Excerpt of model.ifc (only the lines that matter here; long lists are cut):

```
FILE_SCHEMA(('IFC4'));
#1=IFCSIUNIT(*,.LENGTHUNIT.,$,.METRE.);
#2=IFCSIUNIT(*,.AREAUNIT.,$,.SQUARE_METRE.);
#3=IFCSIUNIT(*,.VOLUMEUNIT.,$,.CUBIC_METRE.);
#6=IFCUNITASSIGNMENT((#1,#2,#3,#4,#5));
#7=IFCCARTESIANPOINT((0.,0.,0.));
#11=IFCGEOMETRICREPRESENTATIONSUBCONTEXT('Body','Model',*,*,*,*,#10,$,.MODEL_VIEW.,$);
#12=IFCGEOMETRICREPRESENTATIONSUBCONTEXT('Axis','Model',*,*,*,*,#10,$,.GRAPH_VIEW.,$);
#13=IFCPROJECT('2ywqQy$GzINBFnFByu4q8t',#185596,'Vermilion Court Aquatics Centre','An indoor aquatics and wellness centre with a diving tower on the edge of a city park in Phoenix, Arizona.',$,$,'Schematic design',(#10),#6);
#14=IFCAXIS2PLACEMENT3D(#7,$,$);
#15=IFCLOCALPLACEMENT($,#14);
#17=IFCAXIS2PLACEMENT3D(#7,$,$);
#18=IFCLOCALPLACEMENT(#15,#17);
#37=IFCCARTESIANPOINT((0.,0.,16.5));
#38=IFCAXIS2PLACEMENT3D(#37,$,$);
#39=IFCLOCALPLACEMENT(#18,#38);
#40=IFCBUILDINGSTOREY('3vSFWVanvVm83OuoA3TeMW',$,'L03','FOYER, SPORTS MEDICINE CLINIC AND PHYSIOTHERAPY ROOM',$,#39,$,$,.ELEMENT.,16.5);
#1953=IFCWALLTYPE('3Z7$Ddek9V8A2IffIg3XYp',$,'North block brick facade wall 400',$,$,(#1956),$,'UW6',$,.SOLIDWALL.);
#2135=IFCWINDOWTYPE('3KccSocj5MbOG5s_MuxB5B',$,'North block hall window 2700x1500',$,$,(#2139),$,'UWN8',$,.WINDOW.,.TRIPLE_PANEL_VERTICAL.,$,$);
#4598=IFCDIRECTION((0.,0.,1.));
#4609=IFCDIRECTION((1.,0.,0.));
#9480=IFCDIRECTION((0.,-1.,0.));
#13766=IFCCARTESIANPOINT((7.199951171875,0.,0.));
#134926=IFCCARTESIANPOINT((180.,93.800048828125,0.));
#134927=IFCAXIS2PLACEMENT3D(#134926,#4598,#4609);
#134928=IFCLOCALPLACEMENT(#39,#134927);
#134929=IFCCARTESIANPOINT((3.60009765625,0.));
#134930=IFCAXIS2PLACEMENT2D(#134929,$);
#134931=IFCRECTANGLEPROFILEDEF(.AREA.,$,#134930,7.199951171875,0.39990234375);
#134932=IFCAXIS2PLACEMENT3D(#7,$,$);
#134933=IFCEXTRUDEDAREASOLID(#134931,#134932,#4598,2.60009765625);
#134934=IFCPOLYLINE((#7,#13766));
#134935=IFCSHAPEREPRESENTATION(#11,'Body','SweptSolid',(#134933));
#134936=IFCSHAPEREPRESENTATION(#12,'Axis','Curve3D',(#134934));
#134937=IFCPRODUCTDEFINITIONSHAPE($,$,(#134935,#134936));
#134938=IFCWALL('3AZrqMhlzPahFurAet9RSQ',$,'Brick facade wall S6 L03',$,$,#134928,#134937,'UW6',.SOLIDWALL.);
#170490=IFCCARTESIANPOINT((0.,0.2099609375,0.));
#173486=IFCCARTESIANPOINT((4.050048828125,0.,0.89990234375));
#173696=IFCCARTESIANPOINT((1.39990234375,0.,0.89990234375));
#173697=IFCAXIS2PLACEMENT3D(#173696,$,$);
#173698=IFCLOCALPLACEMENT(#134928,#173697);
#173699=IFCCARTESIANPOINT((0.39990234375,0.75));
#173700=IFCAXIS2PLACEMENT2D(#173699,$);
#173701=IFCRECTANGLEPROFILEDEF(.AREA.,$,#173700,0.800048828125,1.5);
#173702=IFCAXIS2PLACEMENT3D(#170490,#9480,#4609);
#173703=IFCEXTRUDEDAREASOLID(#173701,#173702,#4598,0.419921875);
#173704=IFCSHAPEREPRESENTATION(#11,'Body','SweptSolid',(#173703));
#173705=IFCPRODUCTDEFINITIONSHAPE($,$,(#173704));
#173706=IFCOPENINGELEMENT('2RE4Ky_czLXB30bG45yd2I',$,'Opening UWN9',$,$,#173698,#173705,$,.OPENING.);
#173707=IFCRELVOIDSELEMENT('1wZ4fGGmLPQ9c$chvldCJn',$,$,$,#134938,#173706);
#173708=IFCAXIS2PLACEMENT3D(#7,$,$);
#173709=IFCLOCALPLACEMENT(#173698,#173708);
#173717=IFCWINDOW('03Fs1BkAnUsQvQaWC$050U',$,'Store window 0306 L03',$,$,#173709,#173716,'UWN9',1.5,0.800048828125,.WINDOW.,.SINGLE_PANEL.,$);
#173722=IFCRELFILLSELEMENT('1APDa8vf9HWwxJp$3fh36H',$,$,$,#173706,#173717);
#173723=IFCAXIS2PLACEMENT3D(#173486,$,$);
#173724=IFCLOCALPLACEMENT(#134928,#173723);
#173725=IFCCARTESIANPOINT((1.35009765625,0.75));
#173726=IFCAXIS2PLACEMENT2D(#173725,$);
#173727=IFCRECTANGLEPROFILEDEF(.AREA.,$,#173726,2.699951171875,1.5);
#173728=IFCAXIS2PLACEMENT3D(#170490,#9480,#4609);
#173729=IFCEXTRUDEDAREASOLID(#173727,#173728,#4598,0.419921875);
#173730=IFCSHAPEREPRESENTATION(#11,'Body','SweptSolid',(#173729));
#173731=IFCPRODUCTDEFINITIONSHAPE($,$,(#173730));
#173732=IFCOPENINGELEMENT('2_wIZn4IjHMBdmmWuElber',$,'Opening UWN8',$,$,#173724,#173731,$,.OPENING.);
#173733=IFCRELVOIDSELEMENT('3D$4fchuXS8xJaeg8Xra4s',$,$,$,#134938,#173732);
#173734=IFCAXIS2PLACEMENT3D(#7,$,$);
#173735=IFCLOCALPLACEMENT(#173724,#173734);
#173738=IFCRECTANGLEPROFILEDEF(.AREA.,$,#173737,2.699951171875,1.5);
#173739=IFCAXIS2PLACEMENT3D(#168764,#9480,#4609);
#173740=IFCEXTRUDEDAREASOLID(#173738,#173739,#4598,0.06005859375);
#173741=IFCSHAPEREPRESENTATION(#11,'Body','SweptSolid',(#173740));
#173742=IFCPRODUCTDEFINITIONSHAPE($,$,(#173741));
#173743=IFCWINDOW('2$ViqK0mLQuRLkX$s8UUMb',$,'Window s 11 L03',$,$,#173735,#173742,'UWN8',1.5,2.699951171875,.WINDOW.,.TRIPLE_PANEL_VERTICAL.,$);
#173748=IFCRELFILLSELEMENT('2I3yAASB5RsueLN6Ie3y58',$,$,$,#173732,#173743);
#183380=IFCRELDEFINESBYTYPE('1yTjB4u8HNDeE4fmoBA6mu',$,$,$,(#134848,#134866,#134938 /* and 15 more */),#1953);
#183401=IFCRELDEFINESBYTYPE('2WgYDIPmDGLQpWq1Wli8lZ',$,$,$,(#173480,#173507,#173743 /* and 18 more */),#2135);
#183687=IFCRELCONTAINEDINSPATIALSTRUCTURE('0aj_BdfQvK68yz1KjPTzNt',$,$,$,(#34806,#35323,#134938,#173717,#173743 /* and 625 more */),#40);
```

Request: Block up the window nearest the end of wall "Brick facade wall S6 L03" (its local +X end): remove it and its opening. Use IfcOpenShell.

```python
import ifcopenshell
import ifcopenshell.api.feature
import ifcopenshell.api.root
import ifcopenshell.geom
import ifcopenshell.util.shape

model = ifcopenshell.open("model.ifc")
settings = ifcopenshell.geom.settings()


def volume(element):
    """Net volume in cubic metres, openings subtracted."""
    shape = ifcopenshell.geom.create_shape(settings, element)
    return ifcopenshell.util.shape.get_volume(shape.geometry)


window = model.by_id(173743)
opening = window.FillsVoids[0].RelatingOpeningElement
wall = opening.VoidsElements[0].RelatingBuildingElement
before = volume(wall)

ifcopenshell.api.root.remove_product(model, product=window)
ifcopenshell.api.feature.remove_feature(model, feature=opening)

after = volume(wall)

print(f"wall volume {before:.3f} -> {after:.3f} m3")

model.write("model_edited.ifc")
```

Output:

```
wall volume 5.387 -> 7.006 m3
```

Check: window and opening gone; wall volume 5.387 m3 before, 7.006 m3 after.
